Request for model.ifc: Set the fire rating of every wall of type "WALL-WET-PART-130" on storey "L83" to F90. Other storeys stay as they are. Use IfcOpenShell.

First a look at what the model holds.

```python
import ifcopenshell
import ifcopenshell.util.element

model = ifcopenshell.open("model.ifc")
print(model.schema)
storey = next(s for s in model.by_type("IfcBuildingStorey") if s.Name == "L83")
walls = [e for e in ifcopenshell.util.element.get_decomposition(storey) if e.is_a("IfcWall")]
seen = {}
for e in walls:
    element_type = ifcopenshell.util.element.get_type(e)
    key = (element_type.Name if element_type != e and element_type else None, ifcopenshell.util.element.get_pset(e, "Pset_WallCommon", "FireRating"))
    seen[key] = seen.get(key, 0) + 1
for (name, value), count in sorted(seen.items(), key=str):
    print(count, "x", name, "|", value)
```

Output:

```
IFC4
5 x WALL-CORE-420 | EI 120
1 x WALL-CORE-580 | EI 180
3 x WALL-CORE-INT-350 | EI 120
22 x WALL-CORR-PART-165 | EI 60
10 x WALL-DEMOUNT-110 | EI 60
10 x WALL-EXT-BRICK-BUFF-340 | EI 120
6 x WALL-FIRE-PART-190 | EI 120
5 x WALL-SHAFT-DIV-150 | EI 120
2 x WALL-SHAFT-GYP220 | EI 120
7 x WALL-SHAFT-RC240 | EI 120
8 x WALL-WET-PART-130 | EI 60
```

```python
import ifcopenshell
import ifcopenshell.api.pset
import ifcopenshell.util.element

model = ifcopenshell.open("model.ifc")

storey = next(s for s in model.by_type("IfcBuildingStorey") if s.Name == "L83")
walls = [e for e in ifcopenshell.util.element.get_decomposition(storey) if e.is_a("IfcWall")]

count = 0
for e in walls:
    element_type = ifcopenshell.util.element.get_type(e)
    if element_type in (None, e) or element_type.Name != "WALL-WET-PART-130":
        continue
    found = ifcopenshell.util.element.get_pset(e, "Pset_WallCommon", should_inherit=False)
    if found:
        pset = model.by_id(found["id"])
        if len(ifcopenshell.util.element.get_elements_by_pset(pset)) > 1:
            pset = ifcopenshell.api.pset.unshare_pset(model, products=[e], pset=pset)[0]
    else:
        pset = ifcopenshell.api.pset.add_pset(model, product=e, name="Pset_WallCommon")
    ifcopenshell.api.pset.edit_pset(model, pset=pset, properties={"FireRating": "F90"})
    count += 1

print(count, "walls updated")

model.write("model_edited.ifc")
```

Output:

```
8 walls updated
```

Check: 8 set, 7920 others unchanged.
